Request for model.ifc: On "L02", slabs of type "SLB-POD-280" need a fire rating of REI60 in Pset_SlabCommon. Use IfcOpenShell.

First a look at what the model holds.

```python
import ifcopenshell
import ifcopenshell.util.element

model = ifcopenshell.open("model.ifc")
print(model.schema)
storey = next(s for s in model.by_type("IfcBuildingStorey") if s.Name == "L02")
slabs = [e for e in ifcopenshell.util.element.get_decomposition(storey) if e.is_a("IfcSlab")]
seen = {}
for e in slabs:
    element_type = ifcopenshell.util.element.get_type(e)
    key = (element_type.Name if element_type != e and element_type else None, ifcopenshell.util.element.get_pset(e, "Pset_SlabCommon", "FireRating"))
    seen[key] = seen.get(key, 0) + 1
for (name, value), count in sorted(seen.items(), key=str):
    print(count, "x", name, "|", value)
```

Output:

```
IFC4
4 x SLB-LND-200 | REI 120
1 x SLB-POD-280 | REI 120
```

```python
import ifcopenshell
import ifcopenshell.api.pset
import ifcopenshell.util.element

model = ifcopenshell.open("model.ifc")

storey = next(s for s in model.by_type("IfcBuildingStorey") if s.Name == "L02")
slabs = [e for e in ifcopenshell.util.element.get_decomposition(storey) if e.is_a("IfcSlab")]

count = 0
for e in slabs:
    element_type = ifcopenshell.util.element.get_type(e)
    if element_type in (None, e) or element_type.Name != "SLB-POD-280":
        continue
    found = ifcopenshell.util.element.get_pset(e, "Pset_SlabCommon", should_inherit=False)
    if found:
        pset = model.by_id(found["id"])
        if len(ifcopenshell.util.element.get_elements_by_pset(pset)) > 1:
            pset = ifcopenshell.api.pset.unshare_pset(model, products=[e], pset=pset)[0]
    else:
        pset = ifcopenshell.api.pset.add_pset(model, product=e, name="Pset_SlabCommon")
    ifcopenshell.api.pset.edit_pset(model, pset=pset, properties={"FireRating": "REI60"})
    count += 1

print(count, "slabs updated")

model.write("model_rev.ifc")
```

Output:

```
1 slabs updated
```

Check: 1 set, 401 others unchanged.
